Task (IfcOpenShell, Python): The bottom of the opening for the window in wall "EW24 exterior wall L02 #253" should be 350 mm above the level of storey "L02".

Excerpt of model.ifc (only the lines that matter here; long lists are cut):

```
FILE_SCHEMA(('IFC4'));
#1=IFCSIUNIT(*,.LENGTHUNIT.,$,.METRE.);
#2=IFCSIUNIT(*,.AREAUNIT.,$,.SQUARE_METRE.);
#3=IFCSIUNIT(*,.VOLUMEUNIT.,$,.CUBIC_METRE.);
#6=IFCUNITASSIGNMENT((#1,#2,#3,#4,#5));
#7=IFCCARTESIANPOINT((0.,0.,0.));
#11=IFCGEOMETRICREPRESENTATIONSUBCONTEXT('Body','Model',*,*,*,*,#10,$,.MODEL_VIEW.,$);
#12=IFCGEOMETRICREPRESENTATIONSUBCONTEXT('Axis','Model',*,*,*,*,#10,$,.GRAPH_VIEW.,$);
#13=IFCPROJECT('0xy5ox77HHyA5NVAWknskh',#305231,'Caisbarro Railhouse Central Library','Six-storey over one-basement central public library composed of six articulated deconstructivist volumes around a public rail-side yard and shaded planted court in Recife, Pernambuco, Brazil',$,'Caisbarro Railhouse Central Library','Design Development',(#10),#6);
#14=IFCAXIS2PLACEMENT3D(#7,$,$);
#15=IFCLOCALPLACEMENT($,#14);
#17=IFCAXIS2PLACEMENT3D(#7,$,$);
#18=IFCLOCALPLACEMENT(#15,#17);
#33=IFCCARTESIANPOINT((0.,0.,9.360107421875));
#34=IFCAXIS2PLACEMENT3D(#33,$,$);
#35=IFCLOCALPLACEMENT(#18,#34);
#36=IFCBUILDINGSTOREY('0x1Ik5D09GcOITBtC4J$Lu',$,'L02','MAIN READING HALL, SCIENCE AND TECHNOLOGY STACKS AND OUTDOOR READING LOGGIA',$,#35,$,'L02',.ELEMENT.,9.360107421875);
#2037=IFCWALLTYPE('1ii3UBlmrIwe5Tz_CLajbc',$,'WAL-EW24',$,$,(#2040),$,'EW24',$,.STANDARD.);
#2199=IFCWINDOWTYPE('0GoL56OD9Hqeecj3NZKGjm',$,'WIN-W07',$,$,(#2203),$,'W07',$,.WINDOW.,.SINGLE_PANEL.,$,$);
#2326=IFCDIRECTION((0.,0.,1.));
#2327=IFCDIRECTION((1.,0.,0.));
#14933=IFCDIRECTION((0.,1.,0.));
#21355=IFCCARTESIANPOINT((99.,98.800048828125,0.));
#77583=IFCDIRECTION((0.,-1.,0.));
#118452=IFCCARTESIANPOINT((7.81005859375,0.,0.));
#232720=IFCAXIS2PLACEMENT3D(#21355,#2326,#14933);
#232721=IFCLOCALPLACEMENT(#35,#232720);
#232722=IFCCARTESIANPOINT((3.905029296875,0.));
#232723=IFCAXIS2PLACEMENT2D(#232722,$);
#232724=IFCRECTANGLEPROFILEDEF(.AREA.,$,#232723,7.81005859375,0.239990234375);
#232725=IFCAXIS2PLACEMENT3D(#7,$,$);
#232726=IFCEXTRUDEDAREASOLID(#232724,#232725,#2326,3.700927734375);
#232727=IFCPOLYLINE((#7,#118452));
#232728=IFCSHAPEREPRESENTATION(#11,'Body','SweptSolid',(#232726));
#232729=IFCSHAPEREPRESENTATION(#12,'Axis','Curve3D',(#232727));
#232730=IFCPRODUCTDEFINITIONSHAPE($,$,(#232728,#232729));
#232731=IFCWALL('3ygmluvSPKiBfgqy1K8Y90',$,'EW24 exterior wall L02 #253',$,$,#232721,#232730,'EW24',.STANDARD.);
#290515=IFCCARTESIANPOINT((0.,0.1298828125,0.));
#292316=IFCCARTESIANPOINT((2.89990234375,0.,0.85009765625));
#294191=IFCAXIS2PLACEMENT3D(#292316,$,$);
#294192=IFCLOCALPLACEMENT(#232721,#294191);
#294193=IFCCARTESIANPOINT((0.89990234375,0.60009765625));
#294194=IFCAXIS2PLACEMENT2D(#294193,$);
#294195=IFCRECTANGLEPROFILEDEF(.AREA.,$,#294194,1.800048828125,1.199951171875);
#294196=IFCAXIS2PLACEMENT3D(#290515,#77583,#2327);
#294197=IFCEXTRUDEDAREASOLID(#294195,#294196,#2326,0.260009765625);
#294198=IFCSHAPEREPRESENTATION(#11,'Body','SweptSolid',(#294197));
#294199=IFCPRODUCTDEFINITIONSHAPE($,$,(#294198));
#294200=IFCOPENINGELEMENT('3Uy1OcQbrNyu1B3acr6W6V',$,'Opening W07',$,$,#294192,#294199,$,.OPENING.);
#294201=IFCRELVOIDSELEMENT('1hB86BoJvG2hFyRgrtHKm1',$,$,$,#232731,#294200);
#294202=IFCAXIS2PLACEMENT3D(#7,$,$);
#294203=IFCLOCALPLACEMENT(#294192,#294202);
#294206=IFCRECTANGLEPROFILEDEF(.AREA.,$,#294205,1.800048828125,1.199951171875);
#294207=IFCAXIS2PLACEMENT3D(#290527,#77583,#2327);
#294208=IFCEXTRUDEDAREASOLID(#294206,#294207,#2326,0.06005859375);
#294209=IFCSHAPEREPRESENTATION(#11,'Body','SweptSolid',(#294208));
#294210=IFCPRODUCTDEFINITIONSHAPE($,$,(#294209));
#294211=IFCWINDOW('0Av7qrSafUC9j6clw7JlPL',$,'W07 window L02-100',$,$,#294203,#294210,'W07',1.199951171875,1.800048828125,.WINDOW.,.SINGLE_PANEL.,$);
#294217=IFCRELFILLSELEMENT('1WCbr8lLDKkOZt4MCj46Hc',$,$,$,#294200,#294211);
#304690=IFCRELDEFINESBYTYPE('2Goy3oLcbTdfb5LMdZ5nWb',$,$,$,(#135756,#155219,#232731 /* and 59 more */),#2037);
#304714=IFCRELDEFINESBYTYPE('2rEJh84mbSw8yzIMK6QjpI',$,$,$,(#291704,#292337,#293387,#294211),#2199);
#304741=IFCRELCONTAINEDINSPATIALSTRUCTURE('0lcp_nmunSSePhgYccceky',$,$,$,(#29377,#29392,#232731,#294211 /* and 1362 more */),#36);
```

```python
import numpy as np
import ifcopenshell
import ifcopenshell.api.geometry
import ifcopenshell.geom
import ifcopenshell.util.element
import ifcopenshell.util.placement
import ifcopenshell.util.shape
import ifcopenshell.util.unit

model = ifcopenshell.open("model.ifc")
unit_scale = ifcopenshell.util.unit.calculate_unit_scale(model)

window = model.by_id(294211)
opening = window.FillsVoids[0].RelatingOpeningElement
storey = ifcopenshell.util.element.get_container(window, ifc_class="IfcBuildingStorey")
level = ifcopenshell.util.placement.get_local_placement(storey.ObjectPlacement)[2, 3]

# The opening's origin need not be at the sill, so measure its lowest point.
shape = ifcopenshell.geom.create_shape(ifcopenshell.geom.settings(), opening)
bottom = ifcopenshell.util.shape.get_shape_bottom_elevation(shape, shape.geometry) / unit_scale
dz = level + 0.35 - bottom

shift = np.array([0.0, 0.0, dz])
# The window is placed relative to its opening, so it follows when the opening moves.
matrix = ifcopenshell.util.placement.get_local_placement(opening.ObjectPlacement)
matrix[:3, 3] += shift
ifcopenshell.api.geometry.edit_object_placement(
    model, product=opening, matrix=matrix, is_si=False, should_transform_children=True
)

print(f"moved by {dz * unit_scale:+.3f} m")

model.write("model_updated.ifc")
```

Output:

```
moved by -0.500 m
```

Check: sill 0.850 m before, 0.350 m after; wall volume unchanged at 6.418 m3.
